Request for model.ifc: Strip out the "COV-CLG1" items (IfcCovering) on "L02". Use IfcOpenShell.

First a look at what the model holds.

```python
import ifcopenshell
import ifcopenshell.util.element

model = ifcopenshell.open("model.ifc")
print(model.schema)
storey = next(s for s in model.by_type("IfcBuildingStorey") if s.Name == "L02")
coverings = [e for e in ifcopenshell.util.element.get_decomposition(storey) if e.is_a("IfcCovering")]
seen = {}
for e in coverings:
    element_type = ifcopenshell.util.element.get_type(e)
    name = element_type.Name if element_type not in (None, e) else None
    seen[name] = seen.get(name, 0) + 1
for name, count in sorted(seen.items(), key=str):
    print(count, "x", name)
```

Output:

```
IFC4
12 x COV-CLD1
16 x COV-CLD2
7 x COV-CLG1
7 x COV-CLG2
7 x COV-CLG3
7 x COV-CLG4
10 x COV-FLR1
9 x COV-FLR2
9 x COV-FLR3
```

```python
import ifcopenshell
import ifcopenshell.api.root
import ifcopenshell.util.element

model = ifcopenshell.open("model.ifc")

storey = next(s for s in model.by_type("IfcBuildingStorey") if s.Name == "L02")
coverings = [e for e in ifcopenshell.util.element.get_decomposition(storey) if e.is_a("IfcCovering")]
targets = [e for e in coverings if (t := ifcopenshell.util.element.get_type(e)) not in (None, e) and t.Name == "COV-CLG1"]

for e in targets:
    ifcopenshell.api.root.remove_product(model, product=e)
print(len(targets), "removed")

model.write("model_edited.ifc")
```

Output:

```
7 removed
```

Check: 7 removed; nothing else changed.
